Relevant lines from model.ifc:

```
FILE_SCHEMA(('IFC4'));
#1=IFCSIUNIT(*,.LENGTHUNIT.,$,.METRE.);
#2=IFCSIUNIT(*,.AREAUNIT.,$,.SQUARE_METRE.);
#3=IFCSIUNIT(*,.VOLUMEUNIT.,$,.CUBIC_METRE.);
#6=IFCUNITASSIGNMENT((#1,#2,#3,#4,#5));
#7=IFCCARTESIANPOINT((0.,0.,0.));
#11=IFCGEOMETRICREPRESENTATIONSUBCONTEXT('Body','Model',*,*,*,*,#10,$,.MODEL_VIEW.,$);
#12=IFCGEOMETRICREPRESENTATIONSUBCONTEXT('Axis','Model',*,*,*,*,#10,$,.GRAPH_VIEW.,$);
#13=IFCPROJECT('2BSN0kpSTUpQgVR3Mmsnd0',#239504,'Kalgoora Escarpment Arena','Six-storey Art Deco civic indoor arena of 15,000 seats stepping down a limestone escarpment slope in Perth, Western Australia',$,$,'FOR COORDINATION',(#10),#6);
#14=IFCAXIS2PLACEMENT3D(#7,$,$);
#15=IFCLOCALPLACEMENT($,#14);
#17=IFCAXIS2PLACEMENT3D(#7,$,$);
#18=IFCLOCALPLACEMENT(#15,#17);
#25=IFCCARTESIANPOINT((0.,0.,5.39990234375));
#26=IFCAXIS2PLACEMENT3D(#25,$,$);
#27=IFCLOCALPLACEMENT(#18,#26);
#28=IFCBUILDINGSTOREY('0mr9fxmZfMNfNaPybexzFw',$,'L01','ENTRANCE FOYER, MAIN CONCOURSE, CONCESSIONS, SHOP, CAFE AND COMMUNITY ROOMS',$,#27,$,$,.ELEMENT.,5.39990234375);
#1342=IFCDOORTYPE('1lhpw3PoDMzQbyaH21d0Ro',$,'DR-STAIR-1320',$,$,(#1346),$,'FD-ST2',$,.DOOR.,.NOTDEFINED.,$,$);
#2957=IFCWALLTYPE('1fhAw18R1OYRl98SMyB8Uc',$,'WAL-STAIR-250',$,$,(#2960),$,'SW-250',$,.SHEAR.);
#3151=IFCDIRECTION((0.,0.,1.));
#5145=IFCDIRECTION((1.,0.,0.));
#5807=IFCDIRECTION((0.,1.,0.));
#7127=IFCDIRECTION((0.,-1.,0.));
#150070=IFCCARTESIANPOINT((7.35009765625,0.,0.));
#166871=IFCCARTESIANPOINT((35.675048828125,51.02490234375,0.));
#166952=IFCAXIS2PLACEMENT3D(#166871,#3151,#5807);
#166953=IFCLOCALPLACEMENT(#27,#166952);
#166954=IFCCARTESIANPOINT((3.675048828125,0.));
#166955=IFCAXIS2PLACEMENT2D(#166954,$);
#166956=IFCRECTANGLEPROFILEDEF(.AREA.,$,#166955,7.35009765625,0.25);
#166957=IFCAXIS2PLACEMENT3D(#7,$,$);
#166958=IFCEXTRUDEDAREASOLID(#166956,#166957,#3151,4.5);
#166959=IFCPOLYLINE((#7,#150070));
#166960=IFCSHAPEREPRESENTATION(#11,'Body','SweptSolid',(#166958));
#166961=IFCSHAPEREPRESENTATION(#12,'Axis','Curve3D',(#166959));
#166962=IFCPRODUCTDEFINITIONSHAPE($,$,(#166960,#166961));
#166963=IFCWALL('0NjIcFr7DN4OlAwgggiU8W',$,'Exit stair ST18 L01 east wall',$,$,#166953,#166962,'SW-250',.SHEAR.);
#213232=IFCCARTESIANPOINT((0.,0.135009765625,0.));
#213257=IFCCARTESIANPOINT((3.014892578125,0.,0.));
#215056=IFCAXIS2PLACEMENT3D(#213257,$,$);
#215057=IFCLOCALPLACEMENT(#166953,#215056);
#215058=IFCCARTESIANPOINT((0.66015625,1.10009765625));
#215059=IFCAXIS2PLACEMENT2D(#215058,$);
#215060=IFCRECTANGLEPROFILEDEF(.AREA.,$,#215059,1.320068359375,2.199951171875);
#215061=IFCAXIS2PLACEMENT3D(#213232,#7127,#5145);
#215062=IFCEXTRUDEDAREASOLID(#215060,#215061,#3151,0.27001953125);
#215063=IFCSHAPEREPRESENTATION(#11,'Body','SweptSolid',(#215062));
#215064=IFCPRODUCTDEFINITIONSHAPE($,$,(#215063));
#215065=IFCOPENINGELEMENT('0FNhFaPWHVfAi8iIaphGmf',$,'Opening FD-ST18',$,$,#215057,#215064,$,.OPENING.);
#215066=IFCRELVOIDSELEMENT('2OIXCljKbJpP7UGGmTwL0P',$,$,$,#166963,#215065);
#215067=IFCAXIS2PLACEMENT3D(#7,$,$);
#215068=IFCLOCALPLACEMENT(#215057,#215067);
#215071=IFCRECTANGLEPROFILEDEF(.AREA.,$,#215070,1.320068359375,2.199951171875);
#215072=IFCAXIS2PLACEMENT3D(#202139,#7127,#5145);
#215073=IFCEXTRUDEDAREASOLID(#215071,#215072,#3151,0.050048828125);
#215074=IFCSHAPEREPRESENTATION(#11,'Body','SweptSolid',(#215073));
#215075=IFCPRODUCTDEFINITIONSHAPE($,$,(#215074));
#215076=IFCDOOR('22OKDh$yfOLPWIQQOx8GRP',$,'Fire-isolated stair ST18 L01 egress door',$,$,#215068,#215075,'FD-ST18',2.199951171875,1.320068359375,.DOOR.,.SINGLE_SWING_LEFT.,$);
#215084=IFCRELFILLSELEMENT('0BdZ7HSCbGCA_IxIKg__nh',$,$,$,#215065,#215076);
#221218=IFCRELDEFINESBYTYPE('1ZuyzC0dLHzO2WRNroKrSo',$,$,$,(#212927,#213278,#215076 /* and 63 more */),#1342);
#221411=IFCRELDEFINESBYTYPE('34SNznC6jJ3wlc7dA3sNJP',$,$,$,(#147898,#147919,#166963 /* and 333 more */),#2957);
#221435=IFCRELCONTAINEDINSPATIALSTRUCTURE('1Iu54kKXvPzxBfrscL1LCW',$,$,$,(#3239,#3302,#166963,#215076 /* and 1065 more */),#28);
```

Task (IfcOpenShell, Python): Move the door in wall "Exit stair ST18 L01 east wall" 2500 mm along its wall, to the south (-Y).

```python
import ifcopenshell
import ifcopenshell.api.geometry
import ifcopenshell.util.placement

model = ifcopenshell.open("model.ifc")

door = model.by_guid("22OKDh$yfOLPWIQQOx8GRP")
opening = door.FillsVoids[0].RelatingOpeningElement
wall = opening.VoidsElements[0].RelatingBuildingElement

wall_matrix = ifcopenshell.util.placement.get_local_placement(wall.ObjectPlacement)
shift = wall_matrix[:3, 0] * -2.5
before = ifcopenshell.util.placement.get_local_placement(door.ObjectPlacement)[:3, 3].copy()

# The door is placed relative to its opening, so it follows when the opening moves.
matrix = ifcopenshell.util.placement.get_local_placement(opening.ObjectPlacement)
matrix[:3, 3] += shift
ifcopenshell.api.geometry.edit_object_placement(
    model, product=opening, matrix=matrix, is_si=False, should_transform_children=True
)

after = ifcopenshell.util.placement.get_local_placement(door.ObjectPlacement)[:3, 3]
print("door moved by", (after - before).round(3) + 0.0)

model.write("model_edited.ifc")
```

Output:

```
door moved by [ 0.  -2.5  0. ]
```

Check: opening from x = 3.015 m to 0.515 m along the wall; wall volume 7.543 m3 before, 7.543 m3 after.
